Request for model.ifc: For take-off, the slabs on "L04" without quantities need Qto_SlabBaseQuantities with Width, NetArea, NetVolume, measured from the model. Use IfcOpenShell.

First a look at what the model holds.

```python
import ifcopenshell
import ifcopenshell.util.element
import ifcopenshell.util.unit

model = ifcopenshell.open("model.ifc")
print(model.schema)
for unit_type in ("LENGTHUNIT", "AREAUNIT", "VOLUMEUNIT"):
    print(unit_type, ifcopenshell.util.unit.calculate_unit_scale(model, unit_type))
storey = next(s for s in model.by_type("IfcBuildingStorey") if s.Name == "L04")
slabs = [e for e in ifcopenshell.util.element.get_decomposition(storey) if e.is_a("IfcSlab")]
for e in sorted(slabs, key=lambda e: e.id()):
    print(e.id(), e.is_a(), e.Name, list(ifcopenshell.util.element.get_psets(e, qtos_only=True)), sep=" | ")
```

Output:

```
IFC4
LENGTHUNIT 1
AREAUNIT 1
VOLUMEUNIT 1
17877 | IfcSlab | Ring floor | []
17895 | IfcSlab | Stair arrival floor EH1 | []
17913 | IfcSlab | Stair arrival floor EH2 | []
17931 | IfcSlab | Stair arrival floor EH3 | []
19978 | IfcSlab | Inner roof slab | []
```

```python
import ifcopenshell
import ifcopenshell.api.pset
import ifcopenshell.geom
import ifcopenshell.util.element
import ifcopenshell.util.shape
import ifcopenshell.util.unit

model = ifcopenshell.open("model.ifc")
unit_scale = ifcopenshell.util.unit.calculate_unit_scale(model)
area_scale = ifcopenshell.util.unit.calculate_unit_scale(model, "AREAUNIT")
volume_scale = ifcopenshell.util.unit.calculate_unit_scale(model, "VOLUMEUNIT")
settings = ifcopenshell.geom.settings()

storey = next(s for s in model.by_type("IfcBuildingStorey") if s.Name == "L04")
slabs = [e for e in ifcopenshell.util.element.get_decomposition(storey) if e.is_a("IfcSlab")]

for e in sorted(slabs, key=lambda e: e.id()):
    if ifcopenshell.util.element.get_psets(e, qtos_only=True, should_inherit=False):
        continue
    # Geometry comes back in metres, in the element's own axes.
    shape = ifcopenshell.geom.create_shape(settings, e)
    values = {
        "Width": ifcopenshell.util.shape.get_z(shape.geometry) / unit_scale,
        "NetArea": ifcopenshell.util.shape.get_footprint_area(shape.geometry) / area_scale,
        "NetVolume": ifcopenshell.util.shape.get_volume(shape.geometry) / volume_scale,
    }
    qto = ifcopenshell.api.pset.add_qto(model, product=e, name="Qto_SlabBaseQuantities")
    ifcopenshell.api.pset.edit_qto(model, qto=qto, properties=values)
    print(e.id(), {k: round(v, 3) for k, v in values.items()})

model.write("model_updated.ifc")
```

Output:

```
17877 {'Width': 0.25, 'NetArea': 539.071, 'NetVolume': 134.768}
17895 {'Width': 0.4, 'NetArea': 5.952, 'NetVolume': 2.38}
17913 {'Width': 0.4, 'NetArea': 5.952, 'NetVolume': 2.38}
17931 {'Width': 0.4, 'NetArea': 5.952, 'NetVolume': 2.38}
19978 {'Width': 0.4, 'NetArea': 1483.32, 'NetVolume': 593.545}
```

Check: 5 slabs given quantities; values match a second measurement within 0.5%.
